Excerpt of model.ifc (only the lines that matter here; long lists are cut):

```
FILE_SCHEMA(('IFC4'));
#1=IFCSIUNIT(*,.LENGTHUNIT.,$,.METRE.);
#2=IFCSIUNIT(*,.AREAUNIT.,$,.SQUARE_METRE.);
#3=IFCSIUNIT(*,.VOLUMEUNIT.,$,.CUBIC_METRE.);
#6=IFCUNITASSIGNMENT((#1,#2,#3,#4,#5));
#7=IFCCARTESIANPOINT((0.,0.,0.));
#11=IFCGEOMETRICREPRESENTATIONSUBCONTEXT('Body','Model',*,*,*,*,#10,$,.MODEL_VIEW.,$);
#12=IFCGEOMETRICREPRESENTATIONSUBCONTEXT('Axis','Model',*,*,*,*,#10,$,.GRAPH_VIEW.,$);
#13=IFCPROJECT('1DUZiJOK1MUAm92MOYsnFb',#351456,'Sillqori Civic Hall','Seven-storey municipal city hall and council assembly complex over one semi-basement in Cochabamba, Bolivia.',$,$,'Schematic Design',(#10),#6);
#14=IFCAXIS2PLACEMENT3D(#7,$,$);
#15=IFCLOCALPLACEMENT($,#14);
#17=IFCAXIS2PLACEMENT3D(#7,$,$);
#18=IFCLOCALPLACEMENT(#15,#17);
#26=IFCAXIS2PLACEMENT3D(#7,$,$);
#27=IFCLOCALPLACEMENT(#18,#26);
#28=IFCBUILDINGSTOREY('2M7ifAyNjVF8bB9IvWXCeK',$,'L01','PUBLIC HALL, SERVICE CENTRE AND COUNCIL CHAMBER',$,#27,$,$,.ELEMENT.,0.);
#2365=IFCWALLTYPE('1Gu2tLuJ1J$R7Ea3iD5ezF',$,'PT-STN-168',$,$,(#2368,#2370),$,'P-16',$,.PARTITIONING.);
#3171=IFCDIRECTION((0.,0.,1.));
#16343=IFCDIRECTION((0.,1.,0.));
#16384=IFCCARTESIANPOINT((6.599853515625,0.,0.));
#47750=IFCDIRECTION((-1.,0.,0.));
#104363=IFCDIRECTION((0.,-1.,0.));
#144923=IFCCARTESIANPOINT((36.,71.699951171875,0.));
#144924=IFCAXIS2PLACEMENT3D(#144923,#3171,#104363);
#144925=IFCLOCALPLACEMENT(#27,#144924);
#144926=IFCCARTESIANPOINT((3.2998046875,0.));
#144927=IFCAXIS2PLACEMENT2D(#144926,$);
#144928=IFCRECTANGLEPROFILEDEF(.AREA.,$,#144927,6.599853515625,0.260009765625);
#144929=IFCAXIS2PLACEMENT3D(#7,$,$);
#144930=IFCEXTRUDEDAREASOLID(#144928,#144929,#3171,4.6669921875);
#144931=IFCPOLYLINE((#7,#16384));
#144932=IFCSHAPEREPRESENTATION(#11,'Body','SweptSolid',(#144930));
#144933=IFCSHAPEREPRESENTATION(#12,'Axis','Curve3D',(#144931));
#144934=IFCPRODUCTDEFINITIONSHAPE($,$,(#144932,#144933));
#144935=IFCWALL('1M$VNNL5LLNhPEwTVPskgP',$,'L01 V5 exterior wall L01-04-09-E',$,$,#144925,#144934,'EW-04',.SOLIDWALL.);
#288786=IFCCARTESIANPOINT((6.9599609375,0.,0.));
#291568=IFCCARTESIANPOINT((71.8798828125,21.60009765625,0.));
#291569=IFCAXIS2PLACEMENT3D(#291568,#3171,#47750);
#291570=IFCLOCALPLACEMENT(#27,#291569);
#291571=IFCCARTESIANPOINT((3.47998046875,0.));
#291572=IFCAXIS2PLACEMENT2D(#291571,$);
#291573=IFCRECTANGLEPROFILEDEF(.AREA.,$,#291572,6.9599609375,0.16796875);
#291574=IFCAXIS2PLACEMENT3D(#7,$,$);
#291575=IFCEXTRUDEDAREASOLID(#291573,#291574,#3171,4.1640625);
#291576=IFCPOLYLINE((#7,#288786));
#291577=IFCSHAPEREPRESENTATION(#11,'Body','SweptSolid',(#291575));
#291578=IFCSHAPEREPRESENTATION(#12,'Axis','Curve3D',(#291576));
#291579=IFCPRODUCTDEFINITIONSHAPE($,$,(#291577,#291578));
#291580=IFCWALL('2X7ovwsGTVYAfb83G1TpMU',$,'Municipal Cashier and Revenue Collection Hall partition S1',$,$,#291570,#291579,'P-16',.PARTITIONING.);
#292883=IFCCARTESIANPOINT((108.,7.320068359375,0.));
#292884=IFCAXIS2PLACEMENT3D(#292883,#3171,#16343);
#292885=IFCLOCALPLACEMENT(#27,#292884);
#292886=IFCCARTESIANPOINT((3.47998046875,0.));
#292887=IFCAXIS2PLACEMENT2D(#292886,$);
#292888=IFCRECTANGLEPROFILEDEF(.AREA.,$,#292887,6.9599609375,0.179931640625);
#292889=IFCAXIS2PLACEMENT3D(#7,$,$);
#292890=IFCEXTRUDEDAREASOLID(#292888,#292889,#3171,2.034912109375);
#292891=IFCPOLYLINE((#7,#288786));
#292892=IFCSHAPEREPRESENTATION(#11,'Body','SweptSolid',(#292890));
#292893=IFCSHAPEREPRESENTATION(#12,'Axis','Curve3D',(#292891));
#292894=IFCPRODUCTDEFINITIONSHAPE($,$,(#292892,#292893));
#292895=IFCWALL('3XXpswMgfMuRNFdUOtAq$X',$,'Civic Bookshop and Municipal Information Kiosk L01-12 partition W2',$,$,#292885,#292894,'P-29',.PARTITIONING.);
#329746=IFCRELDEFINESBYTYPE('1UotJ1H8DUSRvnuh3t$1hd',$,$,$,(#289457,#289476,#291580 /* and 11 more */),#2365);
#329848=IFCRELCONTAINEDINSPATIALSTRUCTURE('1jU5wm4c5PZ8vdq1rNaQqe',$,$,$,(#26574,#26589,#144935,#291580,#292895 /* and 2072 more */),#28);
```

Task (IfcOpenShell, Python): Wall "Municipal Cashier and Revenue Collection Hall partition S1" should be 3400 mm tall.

```python
import ifcopenshell
import ifcopenshell.geom
import ifcopenshell.util.representation
import ifcopenshell.util.shape
import ifcopenshell.util.unit

model = ifcopenshell.open("model.ifc")
unit_scale = ifcopenshell.util.unit.calculate_unit_scale(model)
settings = ifcopenshell.geom.settings()


def volume(element):
    """Net volume in cubic metres, openings subtracted."""
    shape = ifcopenshell.geom.create_shape(settings, element)
    return ifcopenshell.util.shape.get_volume(shape.geometry)


wall = model.by_guid("2X7ovwsGTVYAfb83G1TpMU")
before = volume(wall)

body = ifcopenshell.util.representation.get_representation(wall, "Model", "Body")
solid = body.Items[0]
old_height = solid.Depth
solid.Depth = 3.4 / unit_scale
after = volume(wall)

print(f"height {old_height:g} -> {solid.Depth:g}, volume {before:.3f} -> {after:.3f} m3")

model.write("model_edited.ifc")
```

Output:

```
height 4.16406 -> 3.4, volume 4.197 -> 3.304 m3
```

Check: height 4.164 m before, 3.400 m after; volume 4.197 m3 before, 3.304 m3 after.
